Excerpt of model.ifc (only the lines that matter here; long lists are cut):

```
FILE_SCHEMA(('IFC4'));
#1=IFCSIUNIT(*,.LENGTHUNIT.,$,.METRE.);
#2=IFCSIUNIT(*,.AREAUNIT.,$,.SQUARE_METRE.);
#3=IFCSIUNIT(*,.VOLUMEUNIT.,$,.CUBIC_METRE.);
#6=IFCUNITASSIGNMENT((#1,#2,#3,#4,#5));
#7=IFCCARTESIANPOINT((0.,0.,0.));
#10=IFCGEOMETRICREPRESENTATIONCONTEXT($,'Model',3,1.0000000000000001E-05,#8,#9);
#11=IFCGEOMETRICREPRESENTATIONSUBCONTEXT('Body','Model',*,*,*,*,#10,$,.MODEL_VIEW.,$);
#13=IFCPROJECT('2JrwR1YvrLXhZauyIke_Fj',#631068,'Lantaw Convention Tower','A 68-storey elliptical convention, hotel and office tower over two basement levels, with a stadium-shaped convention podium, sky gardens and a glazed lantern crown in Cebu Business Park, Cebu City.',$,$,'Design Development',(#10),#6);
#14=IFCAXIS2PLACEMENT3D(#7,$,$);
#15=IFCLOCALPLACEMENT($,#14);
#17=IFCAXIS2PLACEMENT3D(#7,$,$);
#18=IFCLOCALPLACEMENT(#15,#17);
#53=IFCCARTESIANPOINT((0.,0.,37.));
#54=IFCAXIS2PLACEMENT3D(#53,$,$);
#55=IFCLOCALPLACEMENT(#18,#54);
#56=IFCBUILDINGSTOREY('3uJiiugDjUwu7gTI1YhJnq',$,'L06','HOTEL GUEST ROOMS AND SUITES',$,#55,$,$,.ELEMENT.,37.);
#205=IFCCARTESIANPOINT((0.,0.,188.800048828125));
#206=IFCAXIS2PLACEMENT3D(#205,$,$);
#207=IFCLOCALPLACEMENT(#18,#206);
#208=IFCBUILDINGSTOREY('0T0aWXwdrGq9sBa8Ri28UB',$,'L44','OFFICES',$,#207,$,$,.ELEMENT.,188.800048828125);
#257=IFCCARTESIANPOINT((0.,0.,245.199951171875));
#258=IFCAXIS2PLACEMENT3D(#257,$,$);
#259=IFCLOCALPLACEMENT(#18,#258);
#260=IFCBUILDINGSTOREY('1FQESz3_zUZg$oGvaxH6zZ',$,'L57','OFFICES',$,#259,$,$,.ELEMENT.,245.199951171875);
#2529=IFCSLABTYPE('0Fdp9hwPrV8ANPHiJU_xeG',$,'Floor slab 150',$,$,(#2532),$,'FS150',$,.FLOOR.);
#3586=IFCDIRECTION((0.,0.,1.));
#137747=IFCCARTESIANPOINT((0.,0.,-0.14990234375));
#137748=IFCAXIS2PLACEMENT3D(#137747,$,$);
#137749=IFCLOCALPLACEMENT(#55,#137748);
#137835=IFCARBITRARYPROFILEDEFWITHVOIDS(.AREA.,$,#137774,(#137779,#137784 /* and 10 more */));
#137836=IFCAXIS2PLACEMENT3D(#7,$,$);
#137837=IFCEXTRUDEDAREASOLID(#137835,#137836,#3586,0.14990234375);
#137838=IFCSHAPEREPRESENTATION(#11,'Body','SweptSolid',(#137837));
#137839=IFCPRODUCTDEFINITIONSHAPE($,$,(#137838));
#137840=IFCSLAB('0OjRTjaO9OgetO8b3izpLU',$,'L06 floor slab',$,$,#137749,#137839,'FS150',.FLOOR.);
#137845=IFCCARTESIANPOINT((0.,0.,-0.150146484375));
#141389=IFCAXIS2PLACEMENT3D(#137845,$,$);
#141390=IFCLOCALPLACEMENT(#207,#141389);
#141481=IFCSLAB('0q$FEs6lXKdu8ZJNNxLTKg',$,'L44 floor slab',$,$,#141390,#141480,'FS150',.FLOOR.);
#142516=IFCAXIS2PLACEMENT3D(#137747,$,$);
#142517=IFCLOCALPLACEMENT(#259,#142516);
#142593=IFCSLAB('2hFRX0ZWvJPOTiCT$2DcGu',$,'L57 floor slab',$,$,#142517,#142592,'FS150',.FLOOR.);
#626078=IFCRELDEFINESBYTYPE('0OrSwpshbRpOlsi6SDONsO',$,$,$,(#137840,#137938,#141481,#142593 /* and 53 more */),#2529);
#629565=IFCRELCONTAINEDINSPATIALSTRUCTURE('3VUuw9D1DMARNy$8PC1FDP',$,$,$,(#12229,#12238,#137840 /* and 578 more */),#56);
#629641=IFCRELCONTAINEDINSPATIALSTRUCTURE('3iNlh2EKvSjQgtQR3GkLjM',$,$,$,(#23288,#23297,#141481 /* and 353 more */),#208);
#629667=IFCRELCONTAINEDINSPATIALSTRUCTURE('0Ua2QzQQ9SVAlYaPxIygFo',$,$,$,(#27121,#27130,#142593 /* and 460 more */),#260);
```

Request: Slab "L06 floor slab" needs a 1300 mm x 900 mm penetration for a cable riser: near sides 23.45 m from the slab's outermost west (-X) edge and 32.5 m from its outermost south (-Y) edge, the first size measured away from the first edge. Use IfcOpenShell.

```python
import numpy as np
import ifcopenshell
import ifcopenshell.api.feature
import ifcopenshell.api.geometry
import ifcopenshell.api.root
import ifcopenshell.geom
import ifcopenshell.util.placement
import ifcopenshell.util.representation
import ifcopenshell.util.shape
import ifcopenshell.util.unit

model = ifcopenshell.open("model.ifc")
unit_scale = ifcopenshell.util.unit.calculate_unit_scale(model)
settings = ifcopenshell.geom.settings()


def volume(element):
    """Net volume in cubic metres, openings subtracted."""
    shape = ifcopenshell.geom.create_shape(settings, element)
    return ifcopenshell.util.shape.get_volume(shape.geometry)


slab = model.by_guid("0OjRTjaO9OgetO8b3izpLU")
before = volume(slab)

# Extent in the slab's own axes, in metres. The edges named are its -X and -Y sides.
slab_shape = ifcopenshell.geom.create_shape(settings, slab)
vertices = ifcopenshell.util.shape.get_vertices(slab_shape.geometry)
x_min, y_min, bottom = vertices.min(axis=0)
top = vertices[:, 2].max()

opening = ifcopenshell.api.root.create_entity(model, ifc_class="IfcOpeningElement", name="Cable riser opening", predefined_type="OPENING")
context = ifcopenshell.util.representation.get_context(model, "Model", "Body", "MODEL_VIEW")
width, depth = 1.3, 0.9
outline = [(0.0, 0.0), (width, 0.0), (width, depth), (0.0, depth), (0.0, 0.0)]
# Overshoot both faces by 50 mm so the cut is clean.
shape = ifcopenshell.api.geometry.add_slab_representation(
    model, context=context, depth=top - bottom + 0.1, polyline=outline
)
ifcopenshell.api.geometry.assign_representation(model, product=opening, representation=shape)

matrix = ifcopenshell.util.placement.get_local_placement(slab.ObjectPlacement)
matrix[:, 3] = matrix @ np.append(np.array([x_min + 23.45, y_min + 32.5, bottom - 0.05]) / unit_scale, 1.0)
ifcopenshell.api.geometry.edit_object_placement(model, product=opening, matrix=matrix, is_si=False)
ifcopenshell.api.feature.add_feature(model, feature=opening, element=slab)

after = volume(slab)

print(f"slab volume {before:.3f} -> {after:.3f} m3")

model.write("model-out.ifc")
```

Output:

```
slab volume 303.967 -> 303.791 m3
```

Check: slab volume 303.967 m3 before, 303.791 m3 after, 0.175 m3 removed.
